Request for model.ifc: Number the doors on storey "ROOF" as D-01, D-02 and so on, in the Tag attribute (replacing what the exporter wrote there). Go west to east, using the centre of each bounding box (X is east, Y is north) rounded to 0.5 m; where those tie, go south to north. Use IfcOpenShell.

First a look at what the model holds.

```python
import ifcopenshell
import ifcopenshell.util.element
import ifcopenshell.util.placement

model = ifcopenshell.open("model.ifc")
print(model.schema)
storey = next(s for s in model.by_type("IfcBuildingStorey") if s.Name == "ROOF")
doors = [e for e in ifcopenshell.util.element.get_decomposition(storey) if e.is_a("IfcDoor")]
for e in sorted(doors, key=lambda e: e.id()):
    origin = ifcopenshell.util.placement.get_local_placement(e.ObjectPlacement)[:3, 3]
    print(e.id(), e.Tag, e.Name, origin.round(2) + 0.0, sep=" | ")
```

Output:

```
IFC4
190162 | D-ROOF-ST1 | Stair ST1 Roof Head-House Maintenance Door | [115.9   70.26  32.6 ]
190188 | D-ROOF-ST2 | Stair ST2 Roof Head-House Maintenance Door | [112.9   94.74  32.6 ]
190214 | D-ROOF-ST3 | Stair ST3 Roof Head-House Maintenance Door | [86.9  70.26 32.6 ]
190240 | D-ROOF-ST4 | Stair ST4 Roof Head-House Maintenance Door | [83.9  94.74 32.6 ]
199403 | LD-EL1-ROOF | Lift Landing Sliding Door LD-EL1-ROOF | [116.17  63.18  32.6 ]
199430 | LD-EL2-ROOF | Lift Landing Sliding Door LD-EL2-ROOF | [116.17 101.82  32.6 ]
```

```python
import ifcopenshell
import ifcopenshell.geom
import ifcopenshell.util.element
import ifcopenshell.util.shape

model = ifcopenshell.open("model.ifc")
settings = ifcopenshell.geom.settings()
settings.set("use-world-coords", True)


def centre(element):
    shape = ifcopenshell.geom.create_shape(settings, element)
    return ifcopenshell.util.shape.get_bbox_centroid(shape.geometry)


storey = next(s for s in model.by_type("IfcBuildingStorey") if s.Name == "ROOF")
doors = [e for e in ifcopenshell.util.element.get_decomposition(storey) if e.is_a("IfcDoor")]

# Insertion points can sit at a corner or the storey origin, so sort by the geometry (in metres).
centres = {e: centre(e) for e in doors}
doors.sort(key=lambda e: (round(centres[e][0] / 0.5), centres[e][1]))

for i, e in enumerate(doors, start=1):
    number = f"D-{i:02d}"
    e.Tag = number
    print(e.id(), number)

model.write("model_v2.ifc")
```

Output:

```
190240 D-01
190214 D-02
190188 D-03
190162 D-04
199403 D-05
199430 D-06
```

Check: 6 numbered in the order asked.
